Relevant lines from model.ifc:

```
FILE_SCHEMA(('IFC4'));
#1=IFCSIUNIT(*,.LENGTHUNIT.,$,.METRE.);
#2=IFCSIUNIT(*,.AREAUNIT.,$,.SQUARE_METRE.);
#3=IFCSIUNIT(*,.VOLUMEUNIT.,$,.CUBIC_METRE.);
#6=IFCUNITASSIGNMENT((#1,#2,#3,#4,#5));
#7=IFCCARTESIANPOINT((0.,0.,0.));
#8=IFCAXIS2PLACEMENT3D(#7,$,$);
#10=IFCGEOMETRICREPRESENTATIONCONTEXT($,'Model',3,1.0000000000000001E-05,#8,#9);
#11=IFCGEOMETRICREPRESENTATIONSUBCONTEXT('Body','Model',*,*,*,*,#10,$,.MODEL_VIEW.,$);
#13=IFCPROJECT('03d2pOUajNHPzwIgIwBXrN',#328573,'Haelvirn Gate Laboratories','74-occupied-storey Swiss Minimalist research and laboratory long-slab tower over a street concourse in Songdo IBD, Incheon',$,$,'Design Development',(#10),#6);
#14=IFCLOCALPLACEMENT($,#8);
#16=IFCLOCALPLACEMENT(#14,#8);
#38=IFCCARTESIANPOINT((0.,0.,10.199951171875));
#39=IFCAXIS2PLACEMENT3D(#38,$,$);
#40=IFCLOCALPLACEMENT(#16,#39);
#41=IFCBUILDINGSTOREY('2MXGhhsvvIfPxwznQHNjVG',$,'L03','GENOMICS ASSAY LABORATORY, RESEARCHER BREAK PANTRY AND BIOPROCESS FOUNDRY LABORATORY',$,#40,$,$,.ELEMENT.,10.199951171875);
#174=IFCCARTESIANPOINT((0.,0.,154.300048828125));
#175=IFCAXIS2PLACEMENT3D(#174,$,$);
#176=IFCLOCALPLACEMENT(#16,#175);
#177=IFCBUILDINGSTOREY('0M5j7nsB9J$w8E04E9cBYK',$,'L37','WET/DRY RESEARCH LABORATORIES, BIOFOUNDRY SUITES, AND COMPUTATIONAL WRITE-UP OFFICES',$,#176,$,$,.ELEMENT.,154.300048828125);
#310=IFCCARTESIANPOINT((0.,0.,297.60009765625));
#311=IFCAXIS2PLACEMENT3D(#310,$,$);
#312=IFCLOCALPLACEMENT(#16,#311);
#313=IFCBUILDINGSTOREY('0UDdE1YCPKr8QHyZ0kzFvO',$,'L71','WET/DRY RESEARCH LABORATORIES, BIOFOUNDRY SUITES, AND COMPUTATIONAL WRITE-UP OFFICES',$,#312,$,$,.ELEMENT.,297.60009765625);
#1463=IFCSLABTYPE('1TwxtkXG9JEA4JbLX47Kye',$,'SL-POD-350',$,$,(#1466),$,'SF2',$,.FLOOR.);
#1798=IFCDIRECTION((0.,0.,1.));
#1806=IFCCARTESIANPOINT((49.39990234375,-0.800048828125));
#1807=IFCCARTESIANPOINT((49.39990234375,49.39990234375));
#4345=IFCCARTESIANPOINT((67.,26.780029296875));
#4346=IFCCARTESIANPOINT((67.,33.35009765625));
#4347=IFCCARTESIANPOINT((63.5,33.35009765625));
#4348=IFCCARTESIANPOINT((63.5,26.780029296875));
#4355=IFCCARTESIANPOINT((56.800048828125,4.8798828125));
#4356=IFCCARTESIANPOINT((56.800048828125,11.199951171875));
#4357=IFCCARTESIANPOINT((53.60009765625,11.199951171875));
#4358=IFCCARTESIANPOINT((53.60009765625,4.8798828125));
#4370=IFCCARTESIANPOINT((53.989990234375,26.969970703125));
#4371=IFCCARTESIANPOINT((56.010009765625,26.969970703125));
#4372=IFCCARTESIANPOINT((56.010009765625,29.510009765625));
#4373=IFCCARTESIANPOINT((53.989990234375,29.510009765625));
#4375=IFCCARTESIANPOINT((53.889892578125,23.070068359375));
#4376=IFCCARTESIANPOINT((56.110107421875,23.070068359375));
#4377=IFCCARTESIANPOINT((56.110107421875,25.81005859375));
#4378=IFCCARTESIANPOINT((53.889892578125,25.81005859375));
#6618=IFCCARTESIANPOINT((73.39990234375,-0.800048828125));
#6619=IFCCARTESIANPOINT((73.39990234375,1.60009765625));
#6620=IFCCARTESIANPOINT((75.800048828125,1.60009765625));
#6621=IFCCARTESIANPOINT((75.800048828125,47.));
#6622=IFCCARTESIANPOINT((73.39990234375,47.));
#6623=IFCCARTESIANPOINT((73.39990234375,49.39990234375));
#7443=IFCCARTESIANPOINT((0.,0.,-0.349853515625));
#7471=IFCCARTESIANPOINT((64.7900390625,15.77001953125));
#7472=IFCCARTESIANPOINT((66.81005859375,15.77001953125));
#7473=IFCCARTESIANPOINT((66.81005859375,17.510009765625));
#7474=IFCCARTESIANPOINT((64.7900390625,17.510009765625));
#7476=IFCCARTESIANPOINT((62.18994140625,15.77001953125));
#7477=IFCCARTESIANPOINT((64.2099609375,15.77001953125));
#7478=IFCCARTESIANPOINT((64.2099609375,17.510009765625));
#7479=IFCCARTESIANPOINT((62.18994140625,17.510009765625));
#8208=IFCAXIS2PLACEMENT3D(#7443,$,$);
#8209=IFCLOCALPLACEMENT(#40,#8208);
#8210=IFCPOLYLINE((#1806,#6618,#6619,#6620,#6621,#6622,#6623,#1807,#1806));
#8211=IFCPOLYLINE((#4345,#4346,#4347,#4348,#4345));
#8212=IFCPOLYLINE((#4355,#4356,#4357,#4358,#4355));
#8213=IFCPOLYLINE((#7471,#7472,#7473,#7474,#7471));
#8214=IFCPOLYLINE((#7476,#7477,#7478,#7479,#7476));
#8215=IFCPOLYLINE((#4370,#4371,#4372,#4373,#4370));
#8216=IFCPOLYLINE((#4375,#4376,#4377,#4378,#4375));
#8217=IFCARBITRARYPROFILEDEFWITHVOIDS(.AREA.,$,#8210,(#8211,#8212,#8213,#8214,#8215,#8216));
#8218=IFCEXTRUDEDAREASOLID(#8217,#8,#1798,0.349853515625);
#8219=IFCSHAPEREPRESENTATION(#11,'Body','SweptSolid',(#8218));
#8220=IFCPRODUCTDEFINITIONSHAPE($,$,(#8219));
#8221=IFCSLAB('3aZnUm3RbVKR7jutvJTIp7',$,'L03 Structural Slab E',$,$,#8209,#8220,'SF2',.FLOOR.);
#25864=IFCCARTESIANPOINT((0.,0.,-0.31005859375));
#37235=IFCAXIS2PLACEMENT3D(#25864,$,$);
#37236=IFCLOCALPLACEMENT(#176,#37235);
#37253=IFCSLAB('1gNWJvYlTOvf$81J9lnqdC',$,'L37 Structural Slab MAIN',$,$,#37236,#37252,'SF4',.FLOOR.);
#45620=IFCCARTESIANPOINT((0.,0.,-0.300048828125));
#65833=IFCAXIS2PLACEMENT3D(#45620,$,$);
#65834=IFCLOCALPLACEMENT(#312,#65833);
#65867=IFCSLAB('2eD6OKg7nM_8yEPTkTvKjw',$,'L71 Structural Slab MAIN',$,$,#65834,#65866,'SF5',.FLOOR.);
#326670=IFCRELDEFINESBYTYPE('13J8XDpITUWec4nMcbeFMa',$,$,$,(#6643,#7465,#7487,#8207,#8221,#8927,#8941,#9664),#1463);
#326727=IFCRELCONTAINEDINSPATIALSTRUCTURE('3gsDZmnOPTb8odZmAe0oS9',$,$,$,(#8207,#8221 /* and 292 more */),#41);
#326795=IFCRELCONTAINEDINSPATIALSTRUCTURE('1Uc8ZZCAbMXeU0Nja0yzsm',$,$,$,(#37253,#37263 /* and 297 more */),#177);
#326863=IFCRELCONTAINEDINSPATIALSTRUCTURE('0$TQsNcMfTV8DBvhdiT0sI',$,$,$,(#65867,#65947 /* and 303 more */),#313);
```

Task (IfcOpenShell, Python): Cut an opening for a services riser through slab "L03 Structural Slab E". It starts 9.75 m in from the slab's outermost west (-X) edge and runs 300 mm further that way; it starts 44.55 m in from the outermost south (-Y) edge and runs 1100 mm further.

```python
import numpy as np
import ifcopenshell
import ifcopenshell.api.feature
import ifcopenshell.api.geometry
import ifcopenshell.api.root
import ifcopenshell.geom
import ifcopenshell.util.placement
import ifcopenshell.util.representation
import ifcopenshell.util.shape
import ifcopenshell.util.unit

model = ifcopenshell.open("model.ifc")
unit_scale = ifcopenshell.util.unit.calculate_unit_scale(model)
settings = ifcopenshell.geom.settings()


def volume(element):
    """Net volume in cubic metres, openings subtracted."""
    shape = ifcopenshell.geom.create_shape(settings, element)
    return ifcopenshell.util.shape.get_volume(shape.geometry)


slab = model.by_guid("3aZnUm3RbVKR7jutvJTIp7")
before = volume(slab)

# Extent in the slab's own axes, in metres. The edges named are its -X and -Y sides.
slab_shape = ifcopenshell.geom.create_shape(settings, slab)
vertices = ifcopenshell.util.shape.get_vertices(slab_shape.geometry)
x_min, y_min, bottom = vertices.min(axis=0)
top = vertices[:, 2].max()

opening = ifcopenshell.api.root.create_entity(model, ifc_class="IfcOpeningElement", name="Services riser opening", predefined_type="OPENING")
context = ifcopenshell.util.representation.get_context(model, "Model", "Body", "MODEL_VIEW")
width, depth = 0.3, 1.1
outline = [(0.0, 0.0), (width, 0.0), (width, depth), (0.0, depth), (0.0, 0.0)]
# Overshoot both faces by 50 mm so the cut is clean.
shape = ifcopenshell.api.geometry.add_slab_representation(
    model, context=context, depth=top - bottom + 0.1, polyline=outline
)
ifcopenshell.api.geometry.assign_representation(model, product=opening, representation=shape)

matrix = ifcopenshell.util.placement.get_local_placement(slab.ObjectPlacement)
matrix[:, 3] = matrix @ np.append(np.array([x_min + 9.75, y_min + 44.55, bottom - 0.05]) / unit_scale, 1.0)
ifcopenshell.api.geometry.edit_object_placement(model, product=opening, matrix=matrix, is_si=False)
ifcopenshell.api.feature.add_feature(model, feature=opening, element=slab)

after = volume(slab)

print(f"slab volume {before:.3f} -> {after:.3f} m3")

model.write("model_updated.ifc")
```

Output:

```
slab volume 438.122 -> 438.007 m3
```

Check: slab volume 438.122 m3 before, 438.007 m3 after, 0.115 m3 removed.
